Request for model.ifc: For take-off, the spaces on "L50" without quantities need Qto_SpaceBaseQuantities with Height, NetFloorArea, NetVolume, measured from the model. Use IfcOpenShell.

First a look at what the model holds.

```python
import ifcopenshell
import ifcopenshell.util.element
import ifcopenshell.util.unit

model = ifcopenshell.open("model.ifc")
print(model.schema)
for unit_type in ("LENGTHUNIT", "AREAUNIT", "VOLUMEUNIT"):
    print(unit_type, ifcopenshell.util.unit.calculate_unit_scale(model, unit_type))
storey = next(s for s in model.by_type("IfcBuildingStorey") if s.Name == "L50")
spaces = [e for e in ifcopenshell.util.element.get_decomposition(storey) if e.is_a("IfcSpace")]
for e in sorted(spaces, key=lambda e: e.id()):
    print(e.id(), e.is_a(), e.Name, list(ifcopenshell.util.element.get_psets(e, qtos_only=True)), sep=" | ")
```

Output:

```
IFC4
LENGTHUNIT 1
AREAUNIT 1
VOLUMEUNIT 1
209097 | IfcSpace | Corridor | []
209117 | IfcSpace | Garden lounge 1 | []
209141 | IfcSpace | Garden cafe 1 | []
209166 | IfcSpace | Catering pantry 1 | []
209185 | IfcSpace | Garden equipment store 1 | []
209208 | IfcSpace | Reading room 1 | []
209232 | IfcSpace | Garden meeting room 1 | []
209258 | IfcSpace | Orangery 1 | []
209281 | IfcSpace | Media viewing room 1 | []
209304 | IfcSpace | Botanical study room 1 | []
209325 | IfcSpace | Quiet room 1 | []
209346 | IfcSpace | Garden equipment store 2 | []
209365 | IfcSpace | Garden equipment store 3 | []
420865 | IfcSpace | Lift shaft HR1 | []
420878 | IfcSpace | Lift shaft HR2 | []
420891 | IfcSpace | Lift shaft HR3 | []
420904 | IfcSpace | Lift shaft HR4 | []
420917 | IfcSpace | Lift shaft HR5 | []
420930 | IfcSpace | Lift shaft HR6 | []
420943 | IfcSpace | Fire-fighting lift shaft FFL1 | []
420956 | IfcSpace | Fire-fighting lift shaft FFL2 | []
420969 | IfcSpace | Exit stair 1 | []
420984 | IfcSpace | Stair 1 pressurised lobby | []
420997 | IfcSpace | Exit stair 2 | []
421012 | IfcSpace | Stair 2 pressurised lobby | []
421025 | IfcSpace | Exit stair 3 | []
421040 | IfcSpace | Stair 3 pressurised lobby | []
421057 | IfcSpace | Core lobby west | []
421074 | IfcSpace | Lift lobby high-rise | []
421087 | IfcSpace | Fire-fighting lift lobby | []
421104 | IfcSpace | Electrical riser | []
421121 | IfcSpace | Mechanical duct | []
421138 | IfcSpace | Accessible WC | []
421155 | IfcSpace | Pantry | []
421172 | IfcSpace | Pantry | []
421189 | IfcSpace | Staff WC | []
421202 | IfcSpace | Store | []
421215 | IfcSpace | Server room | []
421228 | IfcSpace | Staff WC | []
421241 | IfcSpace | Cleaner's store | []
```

```python
import ifcopenshell
import ifcopenshell.api.pset
import ifcopenshell.geom
import ifcopenshell.util.element
import ifcopenshell.util.shape
import ifcopenshell.util.unit

model = ifcopenshell.open("model.ifc")
unit_scale = ifcopenshell.util.unit.calculate_unit_scale(model)
area_scale = ifcopenshell.util.unit.calculate_unit_scale(model, "AREAUNIT")
volume_scale = ifcopenshell.util.unit.calculate_unit_scale(model, "VOLUMEUNIT")
settings = ifcopenshell.geom.settings()

storey = next(s for s in model.by_type("IfcBuildingStorey") if s.Name == "L50")
spaces = [e for e in ifcopenshell.util.element.get_decomposition(storey) if e.is_a("IfcSpace")]

for e in sorted(spaces, key=lambda e: e.id()):
    if ifcopenshell.util.element.get_psets(e, qtos_only=True, should_inherit=False):
        continue
    # Geometry comes back in metres, in the element's own axes.
    shape = ifcopenshell.geom.create_shape(settings, e)
    values = {
        "Height": ifcopenshell.util.shape.get_z(shape.geometry) / unit_scale,
        "NetFloorArea": ifcopenshell.util.shape.get_footprint_area(shape.geometry) / area_scale,
        "NetVolume": ifcopenshell.util.shape.get_volume(shape.geometry) / volume_scale,
    }
    qto = ifcopenshell.api.pset.add_qto(model, product=e, name="Qto_SpaceBaseQuantities")
    ifcopenshell.api.pset.edit_qto(model, qto=qto, properties=values)
    print(e.id(), {k: round(v, 3) for k, v in values.items()})

model.write("model_edited.ifc")
```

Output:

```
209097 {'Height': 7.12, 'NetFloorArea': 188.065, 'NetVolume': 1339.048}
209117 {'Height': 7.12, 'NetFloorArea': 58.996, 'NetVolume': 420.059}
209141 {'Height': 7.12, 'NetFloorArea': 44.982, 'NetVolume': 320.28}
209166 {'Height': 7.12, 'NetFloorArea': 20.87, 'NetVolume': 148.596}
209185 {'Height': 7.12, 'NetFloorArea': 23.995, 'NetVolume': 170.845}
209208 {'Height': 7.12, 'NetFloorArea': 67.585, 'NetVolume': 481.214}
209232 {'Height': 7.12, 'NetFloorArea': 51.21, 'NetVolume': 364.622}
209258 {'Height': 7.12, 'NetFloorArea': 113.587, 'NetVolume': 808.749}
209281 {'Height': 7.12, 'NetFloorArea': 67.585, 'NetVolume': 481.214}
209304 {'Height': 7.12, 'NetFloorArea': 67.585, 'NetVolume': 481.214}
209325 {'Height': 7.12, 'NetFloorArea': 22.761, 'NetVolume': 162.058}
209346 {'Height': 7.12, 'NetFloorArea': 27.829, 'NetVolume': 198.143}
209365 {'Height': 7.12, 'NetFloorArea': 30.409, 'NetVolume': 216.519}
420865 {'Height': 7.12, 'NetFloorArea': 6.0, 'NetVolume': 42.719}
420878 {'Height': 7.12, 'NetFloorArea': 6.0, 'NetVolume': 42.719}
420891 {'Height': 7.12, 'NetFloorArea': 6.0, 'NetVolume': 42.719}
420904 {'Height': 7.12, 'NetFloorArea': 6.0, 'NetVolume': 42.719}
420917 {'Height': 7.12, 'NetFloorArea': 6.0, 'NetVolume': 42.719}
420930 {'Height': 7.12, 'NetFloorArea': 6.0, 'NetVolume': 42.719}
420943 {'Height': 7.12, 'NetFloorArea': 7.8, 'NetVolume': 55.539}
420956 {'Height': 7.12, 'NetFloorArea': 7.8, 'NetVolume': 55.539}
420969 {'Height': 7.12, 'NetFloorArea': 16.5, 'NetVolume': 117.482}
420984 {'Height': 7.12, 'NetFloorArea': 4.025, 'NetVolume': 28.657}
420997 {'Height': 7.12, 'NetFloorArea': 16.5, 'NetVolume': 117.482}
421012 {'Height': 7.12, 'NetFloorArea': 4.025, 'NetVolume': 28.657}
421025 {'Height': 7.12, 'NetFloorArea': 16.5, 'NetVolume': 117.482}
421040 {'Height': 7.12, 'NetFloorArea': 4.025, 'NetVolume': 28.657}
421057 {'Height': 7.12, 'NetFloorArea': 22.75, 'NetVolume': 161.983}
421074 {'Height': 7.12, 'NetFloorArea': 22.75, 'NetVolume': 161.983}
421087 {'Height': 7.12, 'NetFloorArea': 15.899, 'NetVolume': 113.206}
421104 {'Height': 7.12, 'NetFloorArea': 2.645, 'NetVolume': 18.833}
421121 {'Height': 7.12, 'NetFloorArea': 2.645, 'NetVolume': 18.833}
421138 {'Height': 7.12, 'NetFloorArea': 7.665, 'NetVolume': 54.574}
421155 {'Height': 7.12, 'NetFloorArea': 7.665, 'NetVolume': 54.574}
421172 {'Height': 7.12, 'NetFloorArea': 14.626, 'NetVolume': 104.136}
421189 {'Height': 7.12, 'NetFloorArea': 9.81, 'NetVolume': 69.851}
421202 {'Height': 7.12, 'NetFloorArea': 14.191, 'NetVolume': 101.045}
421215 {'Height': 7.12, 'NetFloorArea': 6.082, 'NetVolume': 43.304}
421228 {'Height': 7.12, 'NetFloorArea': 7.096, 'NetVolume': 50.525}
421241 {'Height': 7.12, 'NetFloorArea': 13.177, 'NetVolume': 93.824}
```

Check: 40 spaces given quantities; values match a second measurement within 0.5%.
